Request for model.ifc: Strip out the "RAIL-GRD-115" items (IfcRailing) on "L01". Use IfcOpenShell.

First a look at what the model holds.

```python
import ifcopenshell
import ifcopenshell.util.element

model = ifcopenshell.open("model.ifc")
print(model.schema)
storey = next(s for s in model.by_type("IfcBuildingStorey") if s.Name == "L01")
railings = [e for e in ifcopenshell.util.element.get_decomposition(storey) if e.is_a("IfcRailing")]
seen = {}
for e in railings:
    element_type = ifcopenshell.util.element.get_type(e)
    name = element_type.Name if element_type not in (None, e) else None
    seen[name] = seen.get(name, 0) + 1
for name, count in sorted(seen.items(), key=str):
    print(count, "x", name)
```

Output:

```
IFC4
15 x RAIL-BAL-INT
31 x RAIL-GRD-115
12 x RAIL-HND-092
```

```python
import ifcopenshell
import ifcopenshell.api.root
import ifcopenshell.util.element

model = ifcopenshell.open("model.ifc")

storey = next(s for s in model.by_type("IfcBuildingStorey") if s.Name == "L01")
railings = [e for e in ifcopenshell.util.element.get_decomposition(storey) if e.is_a("IfcRailing")]
targets = [e for e in railings if (t := ifcopenshell.util.element.get_type(e)) not in (None, e) and t.Name == "RAIL-GRD-115"]

for e in targets:
    ifcopenshell.api.root.remove_product(model, product=e)
print(len(targets), "removed")

model.write("model_rev.ifc")
```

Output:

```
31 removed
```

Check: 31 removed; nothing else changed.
